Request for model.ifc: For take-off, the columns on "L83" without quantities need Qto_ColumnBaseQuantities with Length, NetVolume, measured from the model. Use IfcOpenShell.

First a look at what the model holds.

```python
import ifcopenshell
import ifcopenshell.util.element
import ifcopenshell.util.unit

model = ifcopenshell.open("model.ifc")
print(model.schema)
for unit_type in ("LENGTHUNIT", "AREAUNIT", "VOLUMEUNIT"):
    print(unit_type, ifcopenshell.util.unit.calculate_unit_scale(model, unit_type))
storey = next(s for s in model.by_type("IfcBuildingStorey") if s.Name == "L83")
columns = [e for e in ifcopenshell.util.element.get_decomposition(storey) if e.is_a("IfcColumn")]
for e in sorted(columns, key=lambda e: e.id()):
    print(e.id(), e.is_a(), e.Name, list(ifcopenshell.util.element.get_psets(e, qtos_only=True)), sep=" | ")
```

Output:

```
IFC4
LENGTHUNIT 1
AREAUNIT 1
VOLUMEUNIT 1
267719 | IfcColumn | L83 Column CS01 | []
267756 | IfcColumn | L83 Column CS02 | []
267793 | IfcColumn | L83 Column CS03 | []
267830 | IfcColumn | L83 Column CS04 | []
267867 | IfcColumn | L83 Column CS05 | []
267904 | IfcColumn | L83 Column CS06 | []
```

```python
import ifcopenshell
import ifcopenshell.api.pset
import ifcopenshell.geom
import ifcopenshell.util.element
import ifcopenshell.util.shape
import ifcopenshell.util.unit

model = ifcopenshell.open("model.ifc")
unit_scale = ifcopenshell.util.unit.calculate_unit_scale(model)
volume_scale = ifcopenshell.util.unit.calculate_unit_scale(model, "VOLUMEUNIT")
settings = ifcopenshell.geom.settings()

storey = next(s for s in model.by_type("IfcBuildingStorey") if s.Name == "L83")
columns = [e for e in ifcopenshell.util.element.get_decomposition(storey) if e.is_a("IfcColumn")]

for e in sorted(columns, key=lambda e: e.id()):
    if ifcopenshell.util.element.get_psets(e, qtos_only=True, should_inherit=False):
        continue
    # Geometry comes back in metres, in the element's own axes.
    shape = ifcopenshell.geom.create_shape(settings, e)
    values = {
        "Length": ifcopenshell.util.shape.get_z(shape.geometry) / unit_scale,
        "NetVolume": ifcopenshell.util.shape.get_volume(shape.geometry) / volume_scale,
    }
    qto = ifcopenshell.api.pset.add_qto(model, product=e, name="Qto_ColumnBaseQuantities")
    ifcopenshell.api.pset.edit_qto(model, qto=qto, properties=values)
    print(e.id(), {k: round(v, 3) for k, v in values.items()})

model.write("model_rev.ifc")
```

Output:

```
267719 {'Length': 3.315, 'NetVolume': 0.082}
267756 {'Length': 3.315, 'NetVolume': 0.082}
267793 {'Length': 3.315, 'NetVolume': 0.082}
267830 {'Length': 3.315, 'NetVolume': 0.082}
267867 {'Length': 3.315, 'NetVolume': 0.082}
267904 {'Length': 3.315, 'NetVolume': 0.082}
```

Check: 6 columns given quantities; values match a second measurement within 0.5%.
